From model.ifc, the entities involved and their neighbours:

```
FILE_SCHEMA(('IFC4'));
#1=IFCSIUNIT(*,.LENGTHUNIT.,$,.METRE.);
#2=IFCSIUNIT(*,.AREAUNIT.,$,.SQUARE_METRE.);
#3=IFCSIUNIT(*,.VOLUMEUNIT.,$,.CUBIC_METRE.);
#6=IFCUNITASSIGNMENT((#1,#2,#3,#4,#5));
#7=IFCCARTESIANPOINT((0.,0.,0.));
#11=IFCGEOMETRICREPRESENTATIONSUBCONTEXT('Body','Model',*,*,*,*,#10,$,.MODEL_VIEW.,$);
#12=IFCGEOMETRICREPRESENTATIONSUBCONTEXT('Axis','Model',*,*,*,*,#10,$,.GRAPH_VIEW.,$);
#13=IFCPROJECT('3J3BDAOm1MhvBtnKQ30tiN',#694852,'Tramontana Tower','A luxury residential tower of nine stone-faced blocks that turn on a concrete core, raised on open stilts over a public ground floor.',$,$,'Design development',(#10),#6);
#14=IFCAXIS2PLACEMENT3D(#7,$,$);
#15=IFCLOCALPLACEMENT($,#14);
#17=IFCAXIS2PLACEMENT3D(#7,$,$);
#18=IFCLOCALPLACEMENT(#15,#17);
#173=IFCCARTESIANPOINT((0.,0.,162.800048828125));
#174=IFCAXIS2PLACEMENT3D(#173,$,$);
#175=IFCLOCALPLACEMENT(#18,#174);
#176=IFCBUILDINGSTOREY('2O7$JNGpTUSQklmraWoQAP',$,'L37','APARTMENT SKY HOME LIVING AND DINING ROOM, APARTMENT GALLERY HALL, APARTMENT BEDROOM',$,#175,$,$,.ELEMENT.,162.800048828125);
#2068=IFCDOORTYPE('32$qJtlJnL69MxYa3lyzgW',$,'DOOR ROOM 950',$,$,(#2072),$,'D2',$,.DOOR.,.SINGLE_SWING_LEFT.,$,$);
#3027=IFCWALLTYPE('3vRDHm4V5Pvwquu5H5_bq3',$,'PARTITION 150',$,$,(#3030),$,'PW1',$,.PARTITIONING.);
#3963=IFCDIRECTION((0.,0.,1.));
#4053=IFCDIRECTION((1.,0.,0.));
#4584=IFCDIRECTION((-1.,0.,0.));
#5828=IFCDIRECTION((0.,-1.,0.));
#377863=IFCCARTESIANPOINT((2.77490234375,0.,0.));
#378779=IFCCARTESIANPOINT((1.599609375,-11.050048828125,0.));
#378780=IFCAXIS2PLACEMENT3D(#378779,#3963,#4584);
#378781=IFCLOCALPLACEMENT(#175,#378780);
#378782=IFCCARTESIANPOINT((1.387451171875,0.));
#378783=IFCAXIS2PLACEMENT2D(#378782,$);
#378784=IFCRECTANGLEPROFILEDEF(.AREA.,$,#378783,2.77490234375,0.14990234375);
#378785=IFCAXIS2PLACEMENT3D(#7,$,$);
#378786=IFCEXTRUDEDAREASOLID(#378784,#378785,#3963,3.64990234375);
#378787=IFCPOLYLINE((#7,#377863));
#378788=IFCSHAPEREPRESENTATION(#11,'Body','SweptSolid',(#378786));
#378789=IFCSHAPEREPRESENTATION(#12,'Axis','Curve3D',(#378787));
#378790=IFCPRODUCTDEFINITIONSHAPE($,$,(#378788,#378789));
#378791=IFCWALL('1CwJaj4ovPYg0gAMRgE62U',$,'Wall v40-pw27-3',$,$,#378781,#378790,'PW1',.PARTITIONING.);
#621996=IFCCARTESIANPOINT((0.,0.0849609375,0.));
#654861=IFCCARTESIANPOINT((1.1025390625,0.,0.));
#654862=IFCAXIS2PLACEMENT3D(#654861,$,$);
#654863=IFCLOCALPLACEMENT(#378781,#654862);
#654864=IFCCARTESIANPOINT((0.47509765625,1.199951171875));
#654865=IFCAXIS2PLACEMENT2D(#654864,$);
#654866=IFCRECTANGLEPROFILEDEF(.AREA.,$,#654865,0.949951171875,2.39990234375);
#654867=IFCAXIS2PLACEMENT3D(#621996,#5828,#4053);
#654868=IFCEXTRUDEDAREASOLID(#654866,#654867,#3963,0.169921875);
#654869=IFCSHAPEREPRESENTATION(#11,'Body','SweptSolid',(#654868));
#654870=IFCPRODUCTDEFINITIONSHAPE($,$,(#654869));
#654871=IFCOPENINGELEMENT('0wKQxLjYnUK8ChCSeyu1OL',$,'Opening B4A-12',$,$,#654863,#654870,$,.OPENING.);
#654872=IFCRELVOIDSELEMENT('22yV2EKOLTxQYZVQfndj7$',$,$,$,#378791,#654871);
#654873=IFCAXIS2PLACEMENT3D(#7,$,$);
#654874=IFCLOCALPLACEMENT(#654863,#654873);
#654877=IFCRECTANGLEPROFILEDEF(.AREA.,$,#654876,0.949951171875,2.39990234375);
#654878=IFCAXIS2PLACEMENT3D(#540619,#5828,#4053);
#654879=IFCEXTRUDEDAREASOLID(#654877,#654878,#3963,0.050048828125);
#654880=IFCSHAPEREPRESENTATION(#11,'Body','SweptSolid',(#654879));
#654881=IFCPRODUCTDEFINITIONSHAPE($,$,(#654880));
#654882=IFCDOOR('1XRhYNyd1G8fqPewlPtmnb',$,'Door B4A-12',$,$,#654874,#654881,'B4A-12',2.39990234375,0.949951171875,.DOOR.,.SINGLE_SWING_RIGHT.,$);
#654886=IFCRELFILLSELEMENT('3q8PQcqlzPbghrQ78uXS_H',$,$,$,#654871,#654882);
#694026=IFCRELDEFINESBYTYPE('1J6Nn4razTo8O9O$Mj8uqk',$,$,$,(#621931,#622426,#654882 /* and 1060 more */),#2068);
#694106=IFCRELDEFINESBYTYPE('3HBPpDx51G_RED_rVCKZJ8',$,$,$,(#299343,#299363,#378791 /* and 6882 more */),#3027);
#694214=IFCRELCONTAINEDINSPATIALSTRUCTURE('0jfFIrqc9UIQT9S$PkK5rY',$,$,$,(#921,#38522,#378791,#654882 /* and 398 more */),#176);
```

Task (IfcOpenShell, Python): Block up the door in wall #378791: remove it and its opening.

```python
import ifcopenshell
import ifcopenshell.api.feature
import ifcopenshell.api.root
import ifcopenshell.geom
import ifcopenshell.util.shape

model = ifcopenshell.open("model.ifc")
settings = ifcopenshell.geom.settings()


def volume(element):
    """Net volume in cubic metres, openings subtracted."""
    shape = ifcopenshell.geom.create_shape(settings, element)
    return ifcopenshell.util.shape.get_volume(shape.geometry)


door = model.by_guid("1XRhYNyd1G8fqPewlPtmnb")
opening = door.FillsVoids[0].RelatingOpeningElement
wall = opening.VoidsElements[0].RelatingBuildingElement
before = volume(wall)

ifcopenshell.api.root.remove_product(model, product=door)
ifcopenshell.api.feature.remove_feature(model, feature=opening)

after = volume(wall)

print(f"wall volume {before:.3f} -> {after:.3f} m3")

model.write("model_rev.ifc")
```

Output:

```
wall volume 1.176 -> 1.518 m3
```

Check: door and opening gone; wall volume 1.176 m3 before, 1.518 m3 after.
